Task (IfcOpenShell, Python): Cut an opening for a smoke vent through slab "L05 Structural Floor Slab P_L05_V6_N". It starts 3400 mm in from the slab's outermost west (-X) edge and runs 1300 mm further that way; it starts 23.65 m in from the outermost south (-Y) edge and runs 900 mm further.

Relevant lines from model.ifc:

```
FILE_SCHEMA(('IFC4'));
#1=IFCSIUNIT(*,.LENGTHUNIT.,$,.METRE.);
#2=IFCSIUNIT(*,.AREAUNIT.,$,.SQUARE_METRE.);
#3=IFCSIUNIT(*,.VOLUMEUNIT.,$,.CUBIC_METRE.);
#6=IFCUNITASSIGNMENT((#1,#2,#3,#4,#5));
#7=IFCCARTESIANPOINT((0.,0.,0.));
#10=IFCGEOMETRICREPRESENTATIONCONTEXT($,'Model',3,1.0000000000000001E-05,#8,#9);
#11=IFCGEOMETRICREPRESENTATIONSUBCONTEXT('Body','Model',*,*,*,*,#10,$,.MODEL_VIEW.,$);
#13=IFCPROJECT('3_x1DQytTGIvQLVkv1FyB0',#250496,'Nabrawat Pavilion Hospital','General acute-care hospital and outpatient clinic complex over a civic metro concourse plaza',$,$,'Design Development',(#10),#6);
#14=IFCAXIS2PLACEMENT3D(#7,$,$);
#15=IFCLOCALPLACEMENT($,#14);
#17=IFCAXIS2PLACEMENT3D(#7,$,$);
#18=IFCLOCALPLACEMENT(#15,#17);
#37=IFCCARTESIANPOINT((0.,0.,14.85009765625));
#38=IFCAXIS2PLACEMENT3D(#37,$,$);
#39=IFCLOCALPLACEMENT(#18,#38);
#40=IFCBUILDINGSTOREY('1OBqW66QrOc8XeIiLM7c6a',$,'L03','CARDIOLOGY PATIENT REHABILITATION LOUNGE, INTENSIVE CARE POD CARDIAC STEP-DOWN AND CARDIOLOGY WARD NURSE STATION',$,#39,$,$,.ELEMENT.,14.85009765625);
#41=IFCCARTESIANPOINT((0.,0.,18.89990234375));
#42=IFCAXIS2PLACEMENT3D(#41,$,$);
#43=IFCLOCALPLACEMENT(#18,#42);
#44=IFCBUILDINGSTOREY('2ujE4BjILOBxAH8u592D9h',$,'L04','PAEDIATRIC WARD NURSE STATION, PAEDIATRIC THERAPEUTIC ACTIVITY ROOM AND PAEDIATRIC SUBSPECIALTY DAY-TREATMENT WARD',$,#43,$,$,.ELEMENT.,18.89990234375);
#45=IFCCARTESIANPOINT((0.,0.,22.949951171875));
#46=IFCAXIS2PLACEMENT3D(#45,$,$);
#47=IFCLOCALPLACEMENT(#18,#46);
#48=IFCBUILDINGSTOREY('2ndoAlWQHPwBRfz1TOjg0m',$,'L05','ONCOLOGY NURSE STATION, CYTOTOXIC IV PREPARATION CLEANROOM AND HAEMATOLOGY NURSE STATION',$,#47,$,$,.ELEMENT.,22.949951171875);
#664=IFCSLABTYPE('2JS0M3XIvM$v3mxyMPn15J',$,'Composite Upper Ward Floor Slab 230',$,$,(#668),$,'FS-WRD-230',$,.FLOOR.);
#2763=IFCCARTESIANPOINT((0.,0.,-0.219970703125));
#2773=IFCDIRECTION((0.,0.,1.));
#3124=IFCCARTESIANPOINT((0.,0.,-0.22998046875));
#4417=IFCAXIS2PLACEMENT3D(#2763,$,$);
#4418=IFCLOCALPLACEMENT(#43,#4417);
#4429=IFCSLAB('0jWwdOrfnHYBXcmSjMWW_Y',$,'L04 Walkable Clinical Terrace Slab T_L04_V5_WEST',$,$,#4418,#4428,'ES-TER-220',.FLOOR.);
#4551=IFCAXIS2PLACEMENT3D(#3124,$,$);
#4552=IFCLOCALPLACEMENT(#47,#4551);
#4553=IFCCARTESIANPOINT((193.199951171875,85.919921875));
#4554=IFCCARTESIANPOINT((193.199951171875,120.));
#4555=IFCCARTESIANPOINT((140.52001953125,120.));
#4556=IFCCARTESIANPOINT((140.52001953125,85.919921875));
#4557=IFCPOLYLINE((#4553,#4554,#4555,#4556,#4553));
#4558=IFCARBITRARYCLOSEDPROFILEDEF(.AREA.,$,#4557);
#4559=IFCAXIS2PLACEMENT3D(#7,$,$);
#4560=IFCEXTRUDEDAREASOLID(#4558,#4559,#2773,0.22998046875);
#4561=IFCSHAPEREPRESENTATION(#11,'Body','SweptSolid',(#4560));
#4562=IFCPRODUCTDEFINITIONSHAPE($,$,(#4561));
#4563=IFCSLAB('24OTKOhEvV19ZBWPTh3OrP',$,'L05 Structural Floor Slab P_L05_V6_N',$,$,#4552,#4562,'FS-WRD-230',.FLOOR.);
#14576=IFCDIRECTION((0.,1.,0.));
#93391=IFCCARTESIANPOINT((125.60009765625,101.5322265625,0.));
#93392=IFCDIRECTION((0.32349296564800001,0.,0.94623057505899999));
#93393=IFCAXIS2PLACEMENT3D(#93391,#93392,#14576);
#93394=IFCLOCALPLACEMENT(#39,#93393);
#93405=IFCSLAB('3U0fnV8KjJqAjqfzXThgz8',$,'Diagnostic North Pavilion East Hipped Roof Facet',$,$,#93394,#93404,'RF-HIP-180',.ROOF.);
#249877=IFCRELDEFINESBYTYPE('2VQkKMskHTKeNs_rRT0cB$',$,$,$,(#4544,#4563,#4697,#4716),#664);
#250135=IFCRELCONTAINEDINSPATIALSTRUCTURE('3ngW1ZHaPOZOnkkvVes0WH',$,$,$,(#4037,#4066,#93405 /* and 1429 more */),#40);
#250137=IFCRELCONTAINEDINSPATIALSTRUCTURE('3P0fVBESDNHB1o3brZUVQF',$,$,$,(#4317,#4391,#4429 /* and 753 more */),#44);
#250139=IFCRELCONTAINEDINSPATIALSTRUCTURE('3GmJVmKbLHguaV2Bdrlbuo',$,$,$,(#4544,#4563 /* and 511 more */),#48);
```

```python
import numpy as np
import ifcopenshell
import ifcopenshell.api.feature
import ifcopenshell.api.geometry
import ifcopenshell.api.root
import ifcopenshell.geom
import ifcopenshell.util.placement
import ifcopenshell.util.representation
import ifcopenshell.util.shape
import ifcopenshell.util.unit

model = ifcopenshell.open("model.ifc")
unit_scale = ifcopenshell.util.unit.calculate_unit_scale(model)
settings = ifcopenshell.geom.settings()


def volume(element):
    """Net volume in cubic metres, openings subtracted."""
    shape = ifcopenshell.geom.create_shape(settings, element)
    return ifcopenshell.util.shape.get_volume(shape.geometry)


slab = model.by_guid("24OTKOhEvV19ZBWPTh3OrP")
before = volume(slab)

# Extent in the slab's own axes, in metres. The edges named are its -X and -Y sides.
slab_shape = ifcopenshell.geom.create_shape(settings, slab)
vertices = ifcopenshell.util.shape.get_vertices(slab_shape.geometry)
x_min, y_min, bottom = vertices.min(axis=0)
top = vertices[:, 2].max()

opening = ifcopenshell.api.root.create_entity(model, ifc_class="IfcOpeningElement", name="Smoke vent opening", predefined_type="OPENING")
context = ifcopenshell.util.representation.get_context(model, "Model", "Body", "MODEL_VIEW")
width, depth = 1.3, 0.9
outline = [(0.0, 0.0), (width, 0.0), (width, depth), (0.0, depth), (0.0, 0.0)]
# Overshoot both faces by 50 mm so the cut is clean.
shape = ifcopenshell.api.geometry.add_slab_representation(
    model, context=context, depth=top - bottom + 0.1, polyline=outline
)
ifcopenshell.api.geometry.assign_representation(model, product=opening, representation=shape)

matrix = ifcopenshell.util.placement.get_local_placement(slab.ObjectPlacement)
matrix[:, 3] = matrix @ np.append(np.array([x_min + 3.4, y_min + 23.65, bottom - 0.05]) / unit_scale, 1.0)
ifcopenshell.api.geometry.edit_object_placement(model, product=opening, matrix=matrix, is_si=False)
ifcopenshell.api.feature.add_feature(model, feature=opening, element=slab)

after = volume(slab)

print(f"slab volume {before:.3f} -> {after:.3f} m3")

model.write("model_v2.ifc")
```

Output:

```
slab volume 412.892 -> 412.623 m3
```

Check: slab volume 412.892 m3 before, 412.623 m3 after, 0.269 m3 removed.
